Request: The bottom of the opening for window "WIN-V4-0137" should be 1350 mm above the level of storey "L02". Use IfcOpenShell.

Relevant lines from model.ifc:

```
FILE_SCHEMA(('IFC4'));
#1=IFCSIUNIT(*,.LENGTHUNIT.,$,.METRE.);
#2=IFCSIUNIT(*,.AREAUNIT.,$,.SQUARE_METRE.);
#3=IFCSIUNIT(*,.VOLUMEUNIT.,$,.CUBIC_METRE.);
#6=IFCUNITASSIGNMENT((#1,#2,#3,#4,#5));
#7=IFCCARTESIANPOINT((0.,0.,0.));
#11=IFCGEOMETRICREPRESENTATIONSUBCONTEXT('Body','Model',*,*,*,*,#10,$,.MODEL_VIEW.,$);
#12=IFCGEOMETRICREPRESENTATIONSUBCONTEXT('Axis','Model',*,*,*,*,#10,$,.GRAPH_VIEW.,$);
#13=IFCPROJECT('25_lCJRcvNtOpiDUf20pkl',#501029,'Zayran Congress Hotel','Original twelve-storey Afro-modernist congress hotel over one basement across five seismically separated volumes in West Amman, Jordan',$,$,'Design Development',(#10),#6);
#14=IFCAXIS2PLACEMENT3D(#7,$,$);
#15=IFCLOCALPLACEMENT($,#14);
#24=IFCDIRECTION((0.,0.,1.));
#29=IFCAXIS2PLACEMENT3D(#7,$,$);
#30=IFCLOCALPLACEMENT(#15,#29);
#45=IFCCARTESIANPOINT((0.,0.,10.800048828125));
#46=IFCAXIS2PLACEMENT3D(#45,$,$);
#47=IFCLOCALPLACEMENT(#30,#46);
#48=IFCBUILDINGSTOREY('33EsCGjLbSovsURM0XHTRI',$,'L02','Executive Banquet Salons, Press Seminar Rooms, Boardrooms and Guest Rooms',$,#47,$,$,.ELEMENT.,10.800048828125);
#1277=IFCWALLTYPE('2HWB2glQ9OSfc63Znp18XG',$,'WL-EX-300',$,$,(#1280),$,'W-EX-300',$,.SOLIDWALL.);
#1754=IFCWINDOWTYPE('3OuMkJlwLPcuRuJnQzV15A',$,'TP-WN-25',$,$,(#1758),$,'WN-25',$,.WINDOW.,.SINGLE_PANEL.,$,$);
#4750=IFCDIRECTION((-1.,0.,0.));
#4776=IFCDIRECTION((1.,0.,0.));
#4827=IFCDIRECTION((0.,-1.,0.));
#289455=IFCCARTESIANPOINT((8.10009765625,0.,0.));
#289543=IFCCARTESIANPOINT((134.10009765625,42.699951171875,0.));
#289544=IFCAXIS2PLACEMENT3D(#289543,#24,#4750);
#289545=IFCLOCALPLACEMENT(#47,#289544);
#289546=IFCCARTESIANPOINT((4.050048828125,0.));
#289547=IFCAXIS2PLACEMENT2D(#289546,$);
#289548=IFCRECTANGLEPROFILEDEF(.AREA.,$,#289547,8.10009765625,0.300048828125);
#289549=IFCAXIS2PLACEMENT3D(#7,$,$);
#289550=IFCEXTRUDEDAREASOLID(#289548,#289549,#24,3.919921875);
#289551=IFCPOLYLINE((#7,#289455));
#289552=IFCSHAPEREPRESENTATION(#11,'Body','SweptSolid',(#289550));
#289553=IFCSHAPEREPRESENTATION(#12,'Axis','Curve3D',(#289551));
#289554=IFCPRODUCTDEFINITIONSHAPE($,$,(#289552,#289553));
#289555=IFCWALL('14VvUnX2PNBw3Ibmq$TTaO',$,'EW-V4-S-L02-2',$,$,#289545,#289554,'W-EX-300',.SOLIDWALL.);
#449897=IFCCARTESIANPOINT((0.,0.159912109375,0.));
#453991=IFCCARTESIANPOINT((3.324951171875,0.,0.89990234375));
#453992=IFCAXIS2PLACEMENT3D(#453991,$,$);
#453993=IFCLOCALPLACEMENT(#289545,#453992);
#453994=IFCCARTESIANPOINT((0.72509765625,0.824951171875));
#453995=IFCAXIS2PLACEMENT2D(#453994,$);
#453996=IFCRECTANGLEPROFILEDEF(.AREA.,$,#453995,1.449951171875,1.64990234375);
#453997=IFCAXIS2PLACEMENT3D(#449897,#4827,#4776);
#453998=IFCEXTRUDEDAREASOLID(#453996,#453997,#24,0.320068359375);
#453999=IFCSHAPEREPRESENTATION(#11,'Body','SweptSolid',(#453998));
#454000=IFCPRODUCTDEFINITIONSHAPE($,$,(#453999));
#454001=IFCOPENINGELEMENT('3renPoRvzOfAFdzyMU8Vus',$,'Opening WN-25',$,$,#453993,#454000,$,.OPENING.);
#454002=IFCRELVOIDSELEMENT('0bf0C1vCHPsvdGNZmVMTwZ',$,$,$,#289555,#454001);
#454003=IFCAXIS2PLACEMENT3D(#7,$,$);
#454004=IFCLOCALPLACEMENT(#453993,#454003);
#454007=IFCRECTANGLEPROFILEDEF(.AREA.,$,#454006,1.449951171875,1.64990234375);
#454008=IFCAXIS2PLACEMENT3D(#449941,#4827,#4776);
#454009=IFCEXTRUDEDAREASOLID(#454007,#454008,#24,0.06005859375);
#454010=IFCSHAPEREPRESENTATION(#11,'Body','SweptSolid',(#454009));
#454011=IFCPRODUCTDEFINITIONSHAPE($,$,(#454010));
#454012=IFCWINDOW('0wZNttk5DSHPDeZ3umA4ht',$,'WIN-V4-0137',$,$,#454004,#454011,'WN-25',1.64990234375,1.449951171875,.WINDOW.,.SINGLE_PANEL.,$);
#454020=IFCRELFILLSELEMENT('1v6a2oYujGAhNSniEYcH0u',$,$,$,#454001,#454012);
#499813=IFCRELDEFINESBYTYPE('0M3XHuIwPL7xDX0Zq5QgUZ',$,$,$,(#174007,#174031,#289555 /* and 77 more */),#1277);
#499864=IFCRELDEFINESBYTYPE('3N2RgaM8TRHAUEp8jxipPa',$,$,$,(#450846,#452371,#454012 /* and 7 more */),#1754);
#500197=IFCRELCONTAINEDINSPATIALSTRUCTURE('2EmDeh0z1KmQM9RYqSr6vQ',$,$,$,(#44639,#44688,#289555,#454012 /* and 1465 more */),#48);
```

```python
import numpy as np
import ifcopenshell
import ifcopenshell.api.geometry
import ifcopenshell.geom
import ifcopenshell.util.element
import ifcopenshell.util.placement
import ifcopenshell.util.shape
import ifcopenshell.util.unit

model = ifcopenshell.open("model.ifc")
unit_scale = ifcopenshell.util.unit.calculate_unit_scale(model)

window = model.by_guid("0wZNttk5DSHPDeZ3umA4ht")
opening = window.FillsVoids[0].RelatingOpeningElement
storey = ifcopenshell.util.element.get_container(window, ifc_class="IfcBuildingStorey")
level = ifcopenshell.util.placement.get_local_placement(storey.ObjectPlacement)[2, 3]

# The opening's origin need not be at the sill, so measure its lowest point.
shape = ifcopenshell.geom.create_shape(ifcopenshell.geom.settings(), opening)
bottom = ifcopenshell.util.shape.get_shape_bottom_elevation(shape, shape.geometry) / unit_scale
dz = level + 1.35 / unit_scale - bottom

shift = np.array([0.0, 0.0, dz])
# The window is placed relative to its opening, so it follows when the opening moves.
matrix = ifcopenshell.util.placement.get_local_placement(opening.ObjectPlacement)
matrix[:3, 3] += shift
ifcopenshell.api.geometry.edit_object_placement(
    model, product=opening, matrix=matrix, is_si=False, should_transform_children=True
)

print(f"moved by {dz * unit_scale:+.3f} m")

model.write("model_v2.ifc")
```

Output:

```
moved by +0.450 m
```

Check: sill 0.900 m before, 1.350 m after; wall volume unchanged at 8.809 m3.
